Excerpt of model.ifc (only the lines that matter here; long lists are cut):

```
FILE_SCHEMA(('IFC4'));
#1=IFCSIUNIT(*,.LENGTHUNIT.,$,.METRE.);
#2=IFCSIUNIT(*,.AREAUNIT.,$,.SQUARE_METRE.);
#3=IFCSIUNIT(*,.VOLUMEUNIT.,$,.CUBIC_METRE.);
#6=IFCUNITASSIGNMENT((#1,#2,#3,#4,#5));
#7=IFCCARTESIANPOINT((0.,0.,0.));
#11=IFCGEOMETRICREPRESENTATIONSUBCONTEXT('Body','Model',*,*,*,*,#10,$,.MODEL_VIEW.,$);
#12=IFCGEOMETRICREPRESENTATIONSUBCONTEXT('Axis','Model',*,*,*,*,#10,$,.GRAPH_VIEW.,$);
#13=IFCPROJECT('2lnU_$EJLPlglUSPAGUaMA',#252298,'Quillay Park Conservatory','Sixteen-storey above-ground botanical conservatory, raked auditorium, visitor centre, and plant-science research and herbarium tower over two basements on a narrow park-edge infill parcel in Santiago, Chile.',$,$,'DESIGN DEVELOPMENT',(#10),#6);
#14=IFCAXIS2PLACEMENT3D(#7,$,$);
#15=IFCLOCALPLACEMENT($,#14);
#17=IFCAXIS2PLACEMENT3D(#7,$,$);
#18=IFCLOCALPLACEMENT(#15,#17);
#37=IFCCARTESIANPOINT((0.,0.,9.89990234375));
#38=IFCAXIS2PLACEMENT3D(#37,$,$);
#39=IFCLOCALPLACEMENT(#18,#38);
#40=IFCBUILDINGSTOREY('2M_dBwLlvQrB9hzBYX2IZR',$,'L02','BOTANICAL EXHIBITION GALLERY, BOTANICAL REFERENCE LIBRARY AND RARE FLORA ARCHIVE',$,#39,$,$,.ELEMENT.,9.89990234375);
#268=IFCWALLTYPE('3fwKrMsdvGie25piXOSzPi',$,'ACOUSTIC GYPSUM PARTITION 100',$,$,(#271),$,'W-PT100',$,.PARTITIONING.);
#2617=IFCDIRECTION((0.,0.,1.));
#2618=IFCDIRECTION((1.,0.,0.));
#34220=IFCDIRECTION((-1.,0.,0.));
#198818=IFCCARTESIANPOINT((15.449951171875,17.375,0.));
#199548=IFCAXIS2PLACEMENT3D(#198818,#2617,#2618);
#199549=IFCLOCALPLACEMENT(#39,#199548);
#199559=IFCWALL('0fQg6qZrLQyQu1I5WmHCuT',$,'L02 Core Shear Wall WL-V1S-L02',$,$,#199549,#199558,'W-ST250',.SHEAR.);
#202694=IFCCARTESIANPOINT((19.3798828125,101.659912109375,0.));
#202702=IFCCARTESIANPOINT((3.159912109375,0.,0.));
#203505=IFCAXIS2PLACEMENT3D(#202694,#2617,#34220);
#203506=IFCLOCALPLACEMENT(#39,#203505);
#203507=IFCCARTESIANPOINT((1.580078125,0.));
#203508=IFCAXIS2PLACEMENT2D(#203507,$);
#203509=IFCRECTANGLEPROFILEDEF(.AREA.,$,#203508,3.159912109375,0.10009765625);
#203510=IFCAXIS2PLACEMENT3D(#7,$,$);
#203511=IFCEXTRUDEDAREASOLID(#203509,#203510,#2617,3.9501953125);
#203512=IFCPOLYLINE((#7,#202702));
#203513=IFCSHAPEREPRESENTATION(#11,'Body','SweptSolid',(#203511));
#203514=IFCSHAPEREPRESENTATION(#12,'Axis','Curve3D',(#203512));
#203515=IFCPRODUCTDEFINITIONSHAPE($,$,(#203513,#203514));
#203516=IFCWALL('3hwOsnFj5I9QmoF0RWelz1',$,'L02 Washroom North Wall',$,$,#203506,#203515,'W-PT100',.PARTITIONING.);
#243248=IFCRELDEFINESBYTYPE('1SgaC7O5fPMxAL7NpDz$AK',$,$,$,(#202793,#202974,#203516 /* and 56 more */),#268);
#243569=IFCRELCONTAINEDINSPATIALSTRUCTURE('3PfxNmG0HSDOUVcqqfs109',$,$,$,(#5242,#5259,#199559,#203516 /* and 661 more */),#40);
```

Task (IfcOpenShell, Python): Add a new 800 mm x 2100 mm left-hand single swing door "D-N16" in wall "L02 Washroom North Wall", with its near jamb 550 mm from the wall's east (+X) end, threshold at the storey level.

```python
import numpy as np
import ifcopenshell
import ifcopenshell.api.feature
import ifcopenshell.api.geometry
import ifcopenshell.api.root
import ifcopenshell.api.spatial
import ifcopenshell.geom
import ifcopenshell.util.element
import ifcopenshell.util.placement
import ifcopenshell.util.representation
import ifcopenshell.util.shape
import ifcopenshell.util.unit

model = ifcopenshell.open("model.ifc")
unit_scale = ifcopenshell.util.unit.calculate_unit_scale(model)
settings = ifcopenshell.geom.settings()


def volume(element):
    """Net volume in cubic metres, openings subtracted."""
    shape = ifcopenshell.geom.create_shape(settings, element)
    return ifcopenshell.util.shape.get_volume(shape.geometry)


wall = model.by_guid("3hwOsnFj5I9QmoF0RWelz1")
storey = ifcopenshell.util.element.get_container(wall, ifc_class="IfcBuildingStorey")
context = ifcopenshell.util.representation.get_context(model, "Model", "Body", "MODEL_VIEW")
before = volume(wall)

width, height, from_end, sill = 0.8, 2.1, 0.55, 0.0  # metres

# The wall runs along its own X axis, and the end named is its -X end.
wall_shape = ifcopenshell.geom.create_shape(settings, wall)
x, y, z = ifcopenshell.util.shape.get_vertices(wall_shape.geometry).T
start = x.min() + from_end
face, thickness = float(y.min()), float(y.max() - y.min())
wall_matrix = ifcopenshell.util.placement.get_local_placement(wall.ObjectPlacement)
level = ifcopenshell.util.placement.get_local_placement(storey.ObjectPlacement)[2, 3]


def in_wall(x, y):
    """Placement at x, y metres in the wall's axes, at sill height."""
    matrix = wall_matrix.copy()
    matrix[:, 3] = wall_matrix @ np.array([x / unit_scale, y / unit_scale, 0.0, 1.0])
    matrix[2, 3] = level + sill / unit_scale
    return matrix


# Opening: a box that overshoots both wall faces by 50 mm.
opening = ifcopenshell.api.root.create_entity(model, ifc_class="IfcOpeningElement", predefined_type="OPENING")
box = ifcopenshell.api.geometry.add_wall_representation(
    model, context=context, length=width, height=height, thickness=thickness + 0.1
)
ifcopenshell.api.geometry.assign_representation(model, product=opening, representation=box)
ifcopenshell.api.geometry.edit_object_placement(model, product=opening, matrix=in_wall(start, face - 0.05), is_si=False)
ifcopenshell.api.feature.add_feature(model, feature=opening, element=wall)

door = ifcopenshell.api.root.create_entity(model, ifc_class="IfcDoor", name="D-N16", predefined_type="DOOR")
door.OverallWidth, door.OverallHeight = width / unit_scale, height / unit_scale
door.OperationType = "SINGLE_SWING_LEFT"
body = ifcopenshell.api.geometry.add_door_representation(
    model,
    context=context,
    overall_width=door.OverallWidth,
    overall_height=door.OverallHeight,
    operation_type="SINGLE_SWING_LEFT",
    lining_properties={"LiningDepth": thickness / unit_scale, "ThresholdDepth": thickness / unit_scale},
)
ifcopenshell.api.geometry.assign_representation(model, product=door, representation=body)
ifcopenshell.api.spatial.assign_container(model, products=[door], relating_structure=storey)
ifcopenshell.api.feature.add_filling(model, opening=opening, element=door)

# The lining spans the wall, so the door starts at the wall face.
ifcopenshell.api.geometry.edit_object_placement(model, product=door, matrix=in_wall(start, face), is_si=False)

after = volume(wall)

print(f"wall volume {before:.3f} -> {after:.3f} m3")

model.write("model_updated.ifc")
```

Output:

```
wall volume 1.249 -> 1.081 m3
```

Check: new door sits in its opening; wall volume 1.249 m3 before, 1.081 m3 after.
